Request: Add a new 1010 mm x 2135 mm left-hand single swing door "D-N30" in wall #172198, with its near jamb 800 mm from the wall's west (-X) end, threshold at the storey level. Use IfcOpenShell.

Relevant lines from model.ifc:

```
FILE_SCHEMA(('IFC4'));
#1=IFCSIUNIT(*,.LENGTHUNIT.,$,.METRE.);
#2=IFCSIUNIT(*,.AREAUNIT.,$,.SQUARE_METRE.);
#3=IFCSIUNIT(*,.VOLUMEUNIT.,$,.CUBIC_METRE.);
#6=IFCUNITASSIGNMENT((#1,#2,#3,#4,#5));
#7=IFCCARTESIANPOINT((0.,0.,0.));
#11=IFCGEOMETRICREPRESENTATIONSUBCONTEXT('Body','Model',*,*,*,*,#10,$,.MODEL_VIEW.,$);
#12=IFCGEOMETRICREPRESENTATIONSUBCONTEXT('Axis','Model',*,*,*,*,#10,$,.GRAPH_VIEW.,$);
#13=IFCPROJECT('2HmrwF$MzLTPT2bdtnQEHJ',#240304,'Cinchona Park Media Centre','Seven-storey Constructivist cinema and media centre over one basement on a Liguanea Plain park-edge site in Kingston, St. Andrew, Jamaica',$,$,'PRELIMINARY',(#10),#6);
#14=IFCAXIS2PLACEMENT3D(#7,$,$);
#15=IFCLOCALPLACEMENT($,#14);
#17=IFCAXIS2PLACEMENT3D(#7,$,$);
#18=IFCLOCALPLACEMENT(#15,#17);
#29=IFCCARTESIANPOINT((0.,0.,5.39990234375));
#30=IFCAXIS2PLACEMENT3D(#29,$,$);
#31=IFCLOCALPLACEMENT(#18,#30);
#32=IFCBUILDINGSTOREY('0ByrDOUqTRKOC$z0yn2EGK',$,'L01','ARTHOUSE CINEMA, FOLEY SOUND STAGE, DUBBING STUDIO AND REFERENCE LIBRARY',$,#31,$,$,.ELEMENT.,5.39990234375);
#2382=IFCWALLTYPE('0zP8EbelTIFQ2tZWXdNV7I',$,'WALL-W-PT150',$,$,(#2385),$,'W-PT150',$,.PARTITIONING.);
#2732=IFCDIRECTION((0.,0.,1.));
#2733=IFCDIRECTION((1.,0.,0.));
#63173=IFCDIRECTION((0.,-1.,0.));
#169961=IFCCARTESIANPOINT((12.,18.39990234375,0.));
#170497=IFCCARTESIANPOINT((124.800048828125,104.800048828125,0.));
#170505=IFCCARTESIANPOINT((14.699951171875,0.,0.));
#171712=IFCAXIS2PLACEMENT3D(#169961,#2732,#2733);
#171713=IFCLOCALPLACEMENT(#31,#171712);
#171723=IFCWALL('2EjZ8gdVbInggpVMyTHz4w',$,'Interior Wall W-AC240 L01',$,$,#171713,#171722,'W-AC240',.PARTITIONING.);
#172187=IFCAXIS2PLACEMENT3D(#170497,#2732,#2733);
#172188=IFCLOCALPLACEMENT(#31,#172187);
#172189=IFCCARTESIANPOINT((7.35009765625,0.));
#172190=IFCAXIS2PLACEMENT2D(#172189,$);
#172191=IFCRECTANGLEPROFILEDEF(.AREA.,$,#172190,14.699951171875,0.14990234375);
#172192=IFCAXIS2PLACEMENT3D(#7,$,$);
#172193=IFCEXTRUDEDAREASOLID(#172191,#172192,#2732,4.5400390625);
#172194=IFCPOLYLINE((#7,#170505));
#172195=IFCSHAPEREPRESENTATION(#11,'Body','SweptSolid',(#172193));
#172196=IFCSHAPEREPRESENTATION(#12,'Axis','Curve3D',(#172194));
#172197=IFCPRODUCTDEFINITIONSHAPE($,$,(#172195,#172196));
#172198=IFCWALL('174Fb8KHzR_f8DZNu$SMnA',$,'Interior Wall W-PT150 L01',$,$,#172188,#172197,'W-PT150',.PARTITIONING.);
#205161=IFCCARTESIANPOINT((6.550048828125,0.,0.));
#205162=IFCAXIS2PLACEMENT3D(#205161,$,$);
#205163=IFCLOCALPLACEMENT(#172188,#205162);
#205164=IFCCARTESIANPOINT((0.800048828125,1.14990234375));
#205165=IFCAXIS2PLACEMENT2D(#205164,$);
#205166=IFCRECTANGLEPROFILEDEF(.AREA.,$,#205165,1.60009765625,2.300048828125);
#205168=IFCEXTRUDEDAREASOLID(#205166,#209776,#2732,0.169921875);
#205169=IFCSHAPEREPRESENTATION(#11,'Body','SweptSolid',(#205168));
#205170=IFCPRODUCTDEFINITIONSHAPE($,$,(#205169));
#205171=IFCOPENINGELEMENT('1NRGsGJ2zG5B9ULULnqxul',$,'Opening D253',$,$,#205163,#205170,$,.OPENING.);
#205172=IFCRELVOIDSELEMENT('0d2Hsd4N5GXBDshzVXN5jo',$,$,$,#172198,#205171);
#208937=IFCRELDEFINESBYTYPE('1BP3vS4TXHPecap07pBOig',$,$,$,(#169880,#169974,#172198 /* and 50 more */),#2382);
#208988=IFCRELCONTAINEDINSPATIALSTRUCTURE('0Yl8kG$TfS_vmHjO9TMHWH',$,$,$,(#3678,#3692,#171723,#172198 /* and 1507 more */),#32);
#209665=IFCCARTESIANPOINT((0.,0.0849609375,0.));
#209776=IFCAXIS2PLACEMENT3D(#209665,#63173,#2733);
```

```python
import numpy as np
import ifcopenshell
import ifcopenshell.api.feature
import ifcopenshell.api.geometry
import ifcopenshell.api.root
import ifcopenshell.api.spatial
import ifcopenshell.geom
import ifcopenshell.util.element
import ifcopenshell.util.placement
import ifcopenshell.util.representation
import ifcopenshell.util.shape
import ifcopenshell.util.unit

model = ifcopenshell.open("model.ifc")
unit_scale = ifcopenshell.util.unit.calculate_unit_scale(model)
settings = ifcopenshell.geom.settings()


def volume(element):
    """Net volume in cubic metres, openings subtracted."""
    shape = ifcopenshell.geom.create_shape(settings, element)
    return ifcopenshell.util.shape.get_volume(shape.geometry)


wall = model.by_guid("174Fb8KHzR_f8DZNu$SMnA")
storey = ifcopenshell.util.element.get_container(wall, ifc_class="IfcBuildingStorey")
context = ifcopenshell.util.representation.get_context(model, "Model", "Body", "MODEL_VIEW")
before = volume(wall)

width, height, from_end, sill = 1.01, 2.135, 0.8, 0.0  # metres

# The wall runs along its own X axis, and the end named is its -X end.
wall_shape = ifcopenshell.geom.create_shape(settings, wall)
x, y, z = ifcopenshell.util.shape.get_vertices(wall_shape.geometry).T
start = x.min() + from_end
face, thickness = float(y.min()), float(y.max() - y.min())
wall_matrix = ifcopenshell.util.placement.get_local_placement(wall.ObjectPlacement)
level = ifcopenshell.util.placement.get_local_placement(storey.ObjectPlacement)[2, 3]


def in_wall(x, y):
    """Placement at x, y metres in the wall's axes, at sill height."""
    matrix = wall_matrix.copy()
    matrix[:, 3] = wall_matrix @ np.array([x / unit_scale, y / unit_scale, 0.0, 1.0])
    matrix[2, 3] = level + sill / unit_scale
    return matrix


# Opening: a box that overshoots both wall faces by 50 mm.
opening = ifcopenshell.api.root.create_entity(model, ifc_class="IfcOpeningElement", predefined_type="OPENING")
box = ifcopenshell.api.geometry.add_wall_representation(
    model, context=context, length=width, height=height, thickness=thickness + 0.1
)
ifcopenshell.api.geometry.assign_representation(model, product=opening, representation=box)
ifcopenshell.api.geometry.edit_object_placement(model, product=opening, matrix=in_wall(start, face - 0.05), is_si=False)
ifcopenshell.api.feature.add_feature(model, feature=opening, element=wall)

door = ifcopenshell.api.root.create_entity(model, ifc_class="IfcDoor", name="D-N30", predefined_type="DOOR")
door.OverallWidth, door.OverallHeight = width / unit_scale, height / unit_scale
door.OperationType = "SINGLE_SWING_LEFT"
body = ifcopenshell.api.geometry.add_door_representation(
    model,
    context=context,
    overall_width=door.OverallWidth,
    overall_height=door.OverallHeight,
    operation_type="SINGLE_SWING_LEFT",
    lining_properties={"LiningDepth": thickness / unit_scale, "ThresholdDepth": thickness / unit_scale},
)
ifcopenshell.api.geometry.assign_representation(model, product=door, representation=body)
ifcopenshell.api.spatial.assign_container(model, products=[door], relating_structure=storey)
ifcopenshell.api.feature.add_filling(model, opening=opening, element=door)

# The lining spans the wall, so the door starts at the wall face.
ifcopenshell.api.geometry.edit_object_placement(model, product=door, matrix=in_wall(start, face), is_si=False)

after = volume(wall)

print(f"wall volume {before:.3f} -> {after:.3f} m3")

model.write("model-out.ifc")
```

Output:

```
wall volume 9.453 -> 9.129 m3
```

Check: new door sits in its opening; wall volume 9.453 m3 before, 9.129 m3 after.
